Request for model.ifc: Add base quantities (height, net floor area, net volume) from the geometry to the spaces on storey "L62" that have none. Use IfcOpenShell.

First a look at what the model holds.

```python
import ifcopenshell
import ifcopenshell.util.element
import ifcopenshell.util.unit

model = ifcopenshell.open("model.ifc")
print(model.schema)
for unit_type in ("LENGTHUNIT", "AREAUNIT", "VOLUMEUNIT"):
    print(unit_type, ifcopenshell.util.unit.calculate_unit_scale(model, unit_type))
storey = next(s for s in model.by_type("IfcBuildingStorey") if s.Name == "L62")
spaces = [e for e in ifcopenshell.util.element.get_decomposition(storey) if e.is_a("IfcSpace")]
for e in sorted(spaces, key=lambda e: e.id()):
    print(e.id(), e.is_a(), e.Name, list(ifcopenshell.util.element.get_psets(e, qtos_only=True)), sep=" | ")
```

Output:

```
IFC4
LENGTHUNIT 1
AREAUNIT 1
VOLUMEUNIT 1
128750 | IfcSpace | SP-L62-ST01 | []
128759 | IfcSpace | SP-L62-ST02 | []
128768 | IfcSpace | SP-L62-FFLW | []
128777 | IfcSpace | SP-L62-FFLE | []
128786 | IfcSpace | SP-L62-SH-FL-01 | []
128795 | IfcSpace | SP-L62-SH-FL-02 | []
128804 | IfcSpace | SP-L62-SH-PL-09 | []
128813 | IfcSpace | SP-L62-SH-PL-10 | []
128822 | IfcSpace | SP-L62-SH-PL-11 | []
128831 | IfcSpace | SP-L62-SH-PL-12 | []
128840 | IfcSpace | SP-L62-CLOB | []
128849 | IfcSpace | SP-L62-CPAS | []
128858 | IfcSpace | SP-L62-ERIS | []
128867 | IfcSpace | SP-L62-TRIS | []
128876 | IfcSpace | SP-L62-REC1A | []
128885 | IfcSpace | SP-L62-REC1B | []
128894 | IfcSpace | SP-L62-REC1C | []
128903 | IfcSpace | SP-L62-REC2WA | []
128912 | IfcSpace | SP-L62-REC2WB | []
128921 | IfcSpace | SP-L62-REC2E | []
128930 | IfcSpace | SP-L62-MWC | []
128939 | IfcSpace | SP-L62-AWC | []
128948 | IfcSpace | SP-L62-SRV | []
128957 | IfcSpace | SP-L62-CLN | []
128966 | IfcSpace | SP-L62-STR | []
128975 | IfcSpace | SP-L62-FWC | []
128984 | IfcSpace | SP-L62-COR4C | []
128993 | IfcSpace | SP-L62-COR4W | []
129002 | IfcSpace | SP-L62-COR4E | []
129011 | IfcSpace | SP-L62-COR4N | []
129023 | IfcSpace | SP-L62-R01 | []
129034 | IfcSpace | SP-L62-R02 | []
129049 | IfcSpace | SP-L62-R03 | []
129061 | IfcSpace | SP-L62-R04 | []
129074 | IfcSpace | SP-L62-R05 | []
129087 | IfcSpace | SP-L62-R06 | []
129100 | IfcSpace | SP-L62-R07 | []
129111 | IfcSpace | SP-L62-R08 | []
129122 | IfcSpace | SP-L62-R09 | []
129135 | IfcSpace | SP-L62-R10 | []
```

```python
import ifcopenshell
import ifcopenshell.api.pset
import ifcopenshell.geom
import ifcopenshell.util.element
import ifcopenshell.util.shape
import ifcopenshell.util.unit

model = ifcopenshell.open("model.ifc")
unit_scale = ifcopenshell.util.unit.calculate_unit_scale(model)
area_scale = ifcopenshell.util.unit.calculate_unit_scale(model, "AREAUNIT")
volume_scale = ifcopenshell.util.unit.calculate_unit_scale(model, "VOLUMEUNIT")
settings = ifcopenshell.geom.settings()

storey = next(s for s in model.by_type("IfcBuildingStorey") if s.Name == "L62")
spaces = [e for e in ifcopenshell.util.element.get_decomposition(storey) if e.is_a("IfcSpace")]

for e in sorted(spaces, key=lambda e: e.id()):
    if ifcopenshell.util.element.get_psets(e, qtos_only=True, should_inherit=False):
        continue
    # Geometry comes back in metres, in the element's own axes.
    shape = ifcopenshell.geom.create_shape(settings, e)
    values = {
        "Height": ifcopenshell.util.shape.get_z(shape.geometry) / unit_scale,
        "NetFloorArea": ifcopenshell.util.shape.get_footprint_area(shape.geometry) / area_scale,
        "NetVolume": ifcopenshell.util.shape.get_volume(shape.geometry) / volume_scale,
    }
    qto = ifcopenshell.api.pset.add_qto(model, product=e, name="Qto_SpaceBaseQuantities")
    ifcopenshell.api.pset.edit_qto(model, qto=qto, properties=values)
    print(e.id(), {k: round(v, 3) for k, v in values.items()})

model.write("model_rev.ifc")
```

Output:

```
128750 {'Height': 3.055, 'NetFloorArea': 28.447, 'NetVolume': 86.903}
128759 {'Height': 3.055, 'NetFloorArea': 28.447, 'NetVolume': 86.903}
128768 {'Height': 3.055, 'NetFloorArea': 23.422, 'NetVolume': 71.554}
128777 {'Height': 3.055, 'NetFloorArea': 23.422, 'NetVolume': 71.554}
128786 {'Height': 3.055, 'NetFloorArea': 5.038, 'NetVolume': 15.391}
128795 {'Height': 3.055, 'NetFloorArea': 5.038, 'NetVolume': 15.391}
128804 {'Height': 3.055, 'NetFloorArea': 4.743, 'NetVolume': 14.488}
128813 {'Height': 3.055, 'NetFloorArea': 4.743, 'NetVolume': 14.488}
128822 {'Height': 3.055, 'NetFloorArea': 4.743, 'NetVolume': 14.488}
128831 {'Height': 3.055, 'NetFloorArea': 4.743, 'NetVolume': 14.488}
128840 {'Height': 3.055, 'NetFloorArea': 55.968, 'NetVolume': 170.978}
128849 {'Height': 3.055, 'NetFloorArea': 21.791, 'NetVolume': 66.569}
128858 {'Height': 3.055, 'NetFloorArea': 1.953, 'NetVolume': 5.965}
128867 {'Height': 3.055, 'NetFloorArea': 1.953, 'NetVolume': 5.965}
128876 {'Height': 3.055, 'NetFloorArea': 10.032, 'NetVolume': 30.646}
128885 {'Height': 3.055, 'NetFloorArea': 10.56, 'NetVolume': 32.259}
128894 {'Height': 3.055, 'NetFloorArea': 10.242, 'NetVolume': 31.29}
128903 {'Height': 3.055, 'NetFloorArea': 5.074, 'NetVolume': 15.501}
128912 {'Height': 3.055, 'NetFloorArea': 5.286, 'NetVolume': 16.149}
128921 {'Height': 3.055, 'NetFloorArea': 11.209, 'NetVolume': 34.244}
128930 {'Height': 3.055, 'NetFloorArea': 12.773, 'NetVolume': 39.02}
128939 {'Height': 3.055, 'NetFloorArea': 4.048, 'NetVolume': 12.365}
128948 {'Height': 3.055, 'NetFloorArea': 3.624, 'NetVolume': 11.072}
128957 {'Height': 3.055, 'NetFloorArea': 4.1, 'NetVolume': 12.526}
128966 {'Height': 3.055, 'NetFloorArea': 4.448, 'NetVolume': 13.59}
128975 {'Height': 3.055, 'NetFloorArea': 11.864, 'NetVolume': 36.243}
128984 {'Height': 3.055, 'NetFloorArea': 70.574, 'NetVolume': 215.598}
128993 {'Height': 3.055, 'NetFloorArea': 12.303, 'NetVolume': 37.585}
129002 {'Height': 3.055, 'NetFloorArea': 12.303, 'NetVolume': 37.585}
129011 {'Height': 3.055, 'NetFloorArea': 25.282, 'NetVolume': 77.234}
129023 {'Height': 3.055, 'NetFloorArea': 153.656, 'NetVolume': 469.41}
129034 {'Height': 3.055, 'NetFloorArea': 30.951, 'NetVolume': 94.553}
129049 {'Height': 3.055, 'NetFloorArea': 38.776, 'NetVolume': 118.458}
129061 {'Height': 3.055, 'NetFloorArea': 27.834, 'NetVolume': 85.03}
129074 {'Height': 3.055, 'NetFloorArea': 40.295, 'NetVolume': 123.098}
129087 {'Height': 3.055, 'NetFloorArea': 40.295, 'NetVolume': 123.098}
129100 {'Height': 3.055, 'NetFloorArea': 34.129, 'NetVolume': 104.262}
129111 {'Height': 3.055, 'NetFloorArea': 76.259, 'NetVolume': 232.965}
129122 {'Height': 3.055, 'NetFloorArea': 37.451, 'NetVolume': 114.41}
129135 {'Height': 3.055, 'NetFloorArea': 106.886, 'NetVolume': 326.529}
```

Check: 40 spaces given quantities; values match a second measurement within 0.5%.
